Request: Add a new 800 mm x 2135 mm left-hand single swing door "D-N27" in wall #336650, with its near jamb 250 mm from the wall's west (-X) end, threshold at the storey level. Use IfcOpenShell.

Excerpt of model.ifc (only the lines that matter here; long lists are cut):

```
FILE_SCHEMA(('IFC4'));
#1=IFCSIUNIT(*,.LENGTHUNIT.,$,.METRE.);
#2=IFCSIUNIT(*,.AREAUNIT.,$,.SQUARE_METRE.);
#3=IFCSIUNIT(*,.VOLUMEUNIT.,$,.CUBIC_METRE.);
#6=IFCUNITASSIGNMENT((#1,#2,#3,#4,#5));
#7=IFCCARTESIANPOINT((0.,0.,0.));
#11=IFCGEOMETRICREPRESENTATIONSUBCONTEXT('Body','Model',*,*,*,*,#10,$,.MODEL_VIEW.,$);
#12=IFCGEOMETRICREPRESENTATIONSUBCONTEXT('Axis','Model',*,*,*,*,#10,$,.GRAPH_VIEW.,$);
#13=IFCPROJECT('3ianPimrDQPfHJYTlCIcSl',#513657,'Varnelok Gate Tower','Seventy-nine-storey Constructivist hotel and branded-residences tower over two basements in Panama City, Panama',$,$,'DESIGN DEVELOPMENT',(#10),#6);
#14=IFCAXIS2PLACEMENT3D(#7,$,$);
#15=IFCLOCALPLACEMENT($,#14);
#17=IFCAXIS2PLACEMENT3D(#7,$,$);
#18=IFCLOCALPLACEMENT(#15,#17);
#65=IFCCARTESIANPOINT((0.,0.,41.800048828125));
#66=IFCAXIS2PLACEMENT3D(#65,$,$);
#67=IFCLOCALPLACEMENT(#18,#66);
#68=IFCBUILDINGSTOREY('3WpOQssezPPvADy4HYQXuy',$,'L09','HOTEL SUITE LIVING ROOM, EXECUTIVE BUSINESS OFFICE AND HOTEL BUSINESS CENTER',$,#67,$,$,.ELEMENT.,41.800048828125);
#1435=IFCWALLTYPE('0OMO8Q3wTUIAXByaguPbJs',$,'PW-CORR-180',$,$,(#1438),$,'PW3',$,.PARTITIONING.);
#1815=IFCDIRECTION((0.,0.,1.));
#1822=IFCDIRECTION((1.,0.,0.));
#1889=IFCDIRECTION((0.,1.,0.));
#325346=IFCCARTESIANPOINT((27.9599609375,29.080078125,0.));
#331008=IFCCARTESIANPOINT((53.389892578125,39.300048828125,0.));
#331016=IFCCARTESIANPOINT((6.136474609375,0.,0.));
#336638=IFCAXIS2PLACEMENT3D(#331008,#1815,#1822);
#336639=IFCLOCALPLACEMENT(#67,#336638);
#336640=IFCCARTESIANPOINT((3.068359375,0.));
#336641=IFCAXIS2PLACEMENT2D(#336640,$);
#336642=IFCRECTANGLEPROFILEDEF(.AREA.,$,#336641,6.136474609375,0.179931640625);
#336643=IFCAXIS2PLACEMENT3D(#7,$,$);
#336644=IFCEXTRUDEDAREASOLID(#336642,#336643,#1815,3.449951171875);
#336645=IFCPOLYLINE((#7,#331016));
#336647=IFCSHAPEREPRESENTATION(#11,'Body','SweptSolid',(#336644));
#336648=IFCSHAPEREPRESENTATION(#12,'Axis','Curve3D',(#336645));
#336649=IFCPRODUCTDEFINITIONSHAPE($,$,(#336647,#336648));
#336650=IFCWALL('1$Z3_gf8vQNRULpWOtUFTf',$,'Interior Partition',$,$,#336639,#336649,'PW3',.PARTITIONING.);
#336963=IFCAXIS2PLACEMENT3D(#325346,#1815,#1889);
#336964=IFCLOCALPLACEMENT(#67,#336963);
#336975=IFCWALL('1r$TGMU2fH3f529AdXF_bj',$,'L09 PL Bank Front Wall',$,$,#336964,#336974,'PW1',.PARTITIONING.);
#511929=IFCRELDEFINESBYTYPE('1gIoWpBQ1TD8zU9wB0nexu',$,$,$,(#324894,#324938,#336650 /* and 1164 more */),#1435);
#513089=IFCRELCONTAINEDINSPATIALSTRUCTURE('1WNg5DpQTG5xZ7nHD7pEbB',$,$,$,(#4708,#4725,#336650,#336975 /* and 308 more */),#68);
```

```python
import numpy as np
import ifcopenshell
import ifcopenshell.api.feature
import ifcopenshell.api.geometry
import ifcopenshell.api.root
import ifcopenshell.api.spatial
import ifcopenshell.geom
import ifcopenshell.util.element
import ifcopenshell.util.placement
import ifcopenshell.util.representation
import ifcopenshell.util.shape
import ifcopenshell.util.unit

model = ifcopenshell.open("model.ifc")
unit_scale = ifcopenshell.util.unit.calculate_unit_scale(model)
settings = ifcopenshell.geom.settings()


def volume(element):
    """Net volume in cubic metres, openings subtracted."""
    shape = ifcopenshell.geom.create_shape(settings, element)
    return ifcopenshell.util.shape.get_volume(shape.geometry)


wall = model.by_guid("1$Z3_gf8vQNRULpWOtUFTf")
storey = ifcopenshell.util.element.get_container(wall, ifc_class="IfcBuildingStorey")
context = ifcopenshell.util.representation.get_context(model, "Model", "Body", "MODEL_VIEW")
before = volume(wall)

width, height, from_end, sill = 0.8, 2.135, 0.25, 0.0  # metres

# The wall runs along its own X axis, and the end named is its -X end.
wall_shape = ifcopenshell.geom.create_shape(settings, wall)
x, y, z = ifcopenshell.util.shape.get_vertices(wall_shape.geometry).T
start = x.min() + from_end
face, thickness = float(y.min()), float(y.max() - y.min())
wall_matrix = ifcopenshell.util.placement.get_local_placement(wall.ObjectPlacement)
level = ifcopenshell.util.placement.get_local_placement(storey.ObjectPlacement)[2, 3]


def in_wall(x, y):
    """Placement at x, y metres in the wall's axes, at sill height."""
    matrix = wall_matrix.copy()
    matrix[:, 3] = wall_matrix @ np.array([x / unit_scale, y / unit_scale, 0.0, 1.0])
    matrix[2, 3] = level + sill / unit_scale
    return matrix


# Opening: a box that overshoots both wall faces by 50 mm.
opening = ifcopenshell.api.root.create_entity(model, ifc_class="IfcOpeningElement", predefined_type="OPENING")
box = ifcopenshell.api.geometry.add_wall_representation(
    model, context=context, length=width, height=height, thickness=thickness + 0.1
)
ifcopenshell.api.geometry.assign_representation(model, product=opening, representation=box)
ifcopenshell.api.geometry.edit_object_placement(model, product=opening, matrix=in_wall(start, face - 0.05), is_si=False)
ifcopenshell.api.feature.add_feature(model, feature=opening, element=wall)

door = ifcopenshell.api.root.create_entity(model, ifc_class="IfcDoor", name="D-N27", predefined_type="DOOR")
door.OverallWidth, door.OverallHeight = width / unit_scale, height / unit_scale
door.OperationType = "SINGLE_SWING_LEFT"
body = ifcopenshell.api.geometry.add_door_representation(
    model,
    context=context,
    overall_width=door.OverallWidth,
    overall_height=door.OverallHeight,
    operation_type="SINGLE_SWING_LEFT",
    lining_properties={"LiningDepth": thickness / unit_scale, "ThresholdDepth": thickness / unit_scale},
)
ifcopenshell.api.geometry.assign_representation(model, product=door, representation=body)
ifcopenshell.api.spatial.assign_container(model, products=[door], relating_structure=storey)
ifcopenshell.api.feature.add_filling(model, opening=opening, element=door)

# The lining spans the wall, so the door starts at the wall face.
ifcopenshell.api.geometry.edit_object_placement(model, product=door, matrix=in_wall(start, face), is_si=False)

after = volume(wall)

print(f"wall volume {before:.3f} -> {after:.3f} m3")

model.write("model-out.ifc")
```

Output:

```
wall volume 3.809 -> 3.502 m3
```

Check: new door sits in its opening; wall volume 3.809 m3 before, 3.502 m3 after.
